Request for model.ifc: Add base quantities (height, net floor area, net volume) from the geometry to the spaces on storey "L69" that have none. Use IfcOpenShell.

First a look at what the model holds.

```python
import ifcopenshell
import ifcopenshell.util.element
import ifcopenshell.util.unit

model = ifcopenshell.open("model.ifc")
print(model.schema)
for unit_type in ("LENGTHUNIT", "AREAUNIT", "VOLUMEUNIT"):
    print(unit_type, ifcopenshell.util.unit.calculate_unit_scale(model, unit_type))
storey = next(s for s in model.by_type("IfcBuildingStorey") if s.Name == "L69")
spaces = [e for e in ifcopenshell.util.element.get_decomposition(storey) if e.is_a("IfcSpace")]
for e in sorted(spaces, key=lambda e: e.id()):
    print(e.id(), e.is_a(), e.Name, list(ifcopenshell.util.element.get_psets(e, qtos_only=True)), sep=" | ")
```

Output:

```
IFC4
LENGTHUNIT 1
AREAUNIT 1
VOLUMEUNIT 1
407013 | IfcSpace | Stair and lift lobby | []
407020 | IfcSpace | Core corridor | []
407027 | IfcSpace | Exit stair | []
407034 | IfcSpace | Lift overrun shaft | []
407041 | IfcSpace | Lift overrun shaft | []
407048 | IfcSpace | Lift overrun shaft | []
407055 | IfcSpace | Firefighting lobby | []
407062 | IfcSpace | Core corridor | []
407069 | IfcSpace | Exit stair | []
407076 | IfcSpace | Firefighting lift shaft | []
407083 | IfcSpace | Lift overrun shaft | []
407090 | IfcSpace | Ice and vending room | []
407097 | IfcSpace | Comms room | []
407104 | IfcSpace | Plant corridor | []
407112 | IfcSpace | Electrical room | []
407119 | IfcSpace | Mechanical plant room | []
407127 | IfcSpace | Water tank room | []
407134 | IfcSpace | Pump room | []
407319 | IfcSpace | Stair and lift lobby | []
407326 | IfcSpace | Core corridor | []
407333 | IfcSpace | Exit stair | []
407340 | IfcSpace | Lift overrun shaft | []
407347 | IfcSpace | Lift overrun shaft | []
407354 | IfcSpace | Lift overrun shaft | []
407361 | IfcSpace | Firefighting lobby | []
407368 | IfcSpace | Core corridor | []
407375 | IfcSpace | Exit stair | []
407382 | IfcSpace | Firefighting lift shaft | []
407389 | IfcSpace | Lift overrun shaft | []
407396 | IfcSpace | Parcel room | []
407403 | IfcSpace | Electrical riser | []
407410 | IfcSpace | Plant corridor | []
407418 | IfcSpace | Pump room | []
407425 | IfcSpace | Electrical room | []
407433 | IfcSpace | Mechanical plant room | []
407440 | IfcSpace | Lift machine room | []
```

```python
import ifcopenshell
import ifcopenshell.api.pset
import ifcopenshell.geom
import ifcopenshell.util.element
import ifcopenshell.util.shape
import ifcopenshell.util.unit

model = ifcopenshell.open("model.ifc")
unit_scale = ifcopenshell.util.unit.calculate_unit_scale(model)
area_scale = ifcopenshell.util.unit.calculate_unit_scale(model, "AREAUNIT")
volume_scale = ifcopenshell.util.unit.calculate_unit_scale(model, "VOLUMEUNIT")
settings = ifcopenshell.geom.settings()

storey = next(s for s in model.by_type("IfcBuildingStorey") if s.Name == "L69")
spaces = [e for e in ifcopenshell.util.element.get_decomposition(storey) if e.is_a("IfcSpace")]

for e in sorted(spaces, key=lambda e: e.id()):
    if ifcopenshell.util.element.get_psets(e, qtos_only=True, should_inherit=False):
        continue
    # Geometry comes back in metres, in the element's own axes.
    shape = ifcopenshell.geom.create_shape(settings, e)
    values = {
        "Height": ifcopenshell.util.shape.get_z(shape.geometry) / unit_scale,
        "NetFloorArea": ifcopenshell.util.shape.get_footprint_area(shape.geometry) / area_scale,
        "NetVolume": ifcopenshell.util.shape.get_volume(shape.geometry) / volume_scale,
    }
    qto = ifcopenshell.api.pset.add_qto(model, product=e, name="Qto_SpaceBaseQuantities")
    ifcopenshell.api.pset.edit_qto(model, qto=qto, properties=values)
    print(e.id(), {k: round(v, 3) for k, v in values.items()})

model.write("model_updated.ifc")
```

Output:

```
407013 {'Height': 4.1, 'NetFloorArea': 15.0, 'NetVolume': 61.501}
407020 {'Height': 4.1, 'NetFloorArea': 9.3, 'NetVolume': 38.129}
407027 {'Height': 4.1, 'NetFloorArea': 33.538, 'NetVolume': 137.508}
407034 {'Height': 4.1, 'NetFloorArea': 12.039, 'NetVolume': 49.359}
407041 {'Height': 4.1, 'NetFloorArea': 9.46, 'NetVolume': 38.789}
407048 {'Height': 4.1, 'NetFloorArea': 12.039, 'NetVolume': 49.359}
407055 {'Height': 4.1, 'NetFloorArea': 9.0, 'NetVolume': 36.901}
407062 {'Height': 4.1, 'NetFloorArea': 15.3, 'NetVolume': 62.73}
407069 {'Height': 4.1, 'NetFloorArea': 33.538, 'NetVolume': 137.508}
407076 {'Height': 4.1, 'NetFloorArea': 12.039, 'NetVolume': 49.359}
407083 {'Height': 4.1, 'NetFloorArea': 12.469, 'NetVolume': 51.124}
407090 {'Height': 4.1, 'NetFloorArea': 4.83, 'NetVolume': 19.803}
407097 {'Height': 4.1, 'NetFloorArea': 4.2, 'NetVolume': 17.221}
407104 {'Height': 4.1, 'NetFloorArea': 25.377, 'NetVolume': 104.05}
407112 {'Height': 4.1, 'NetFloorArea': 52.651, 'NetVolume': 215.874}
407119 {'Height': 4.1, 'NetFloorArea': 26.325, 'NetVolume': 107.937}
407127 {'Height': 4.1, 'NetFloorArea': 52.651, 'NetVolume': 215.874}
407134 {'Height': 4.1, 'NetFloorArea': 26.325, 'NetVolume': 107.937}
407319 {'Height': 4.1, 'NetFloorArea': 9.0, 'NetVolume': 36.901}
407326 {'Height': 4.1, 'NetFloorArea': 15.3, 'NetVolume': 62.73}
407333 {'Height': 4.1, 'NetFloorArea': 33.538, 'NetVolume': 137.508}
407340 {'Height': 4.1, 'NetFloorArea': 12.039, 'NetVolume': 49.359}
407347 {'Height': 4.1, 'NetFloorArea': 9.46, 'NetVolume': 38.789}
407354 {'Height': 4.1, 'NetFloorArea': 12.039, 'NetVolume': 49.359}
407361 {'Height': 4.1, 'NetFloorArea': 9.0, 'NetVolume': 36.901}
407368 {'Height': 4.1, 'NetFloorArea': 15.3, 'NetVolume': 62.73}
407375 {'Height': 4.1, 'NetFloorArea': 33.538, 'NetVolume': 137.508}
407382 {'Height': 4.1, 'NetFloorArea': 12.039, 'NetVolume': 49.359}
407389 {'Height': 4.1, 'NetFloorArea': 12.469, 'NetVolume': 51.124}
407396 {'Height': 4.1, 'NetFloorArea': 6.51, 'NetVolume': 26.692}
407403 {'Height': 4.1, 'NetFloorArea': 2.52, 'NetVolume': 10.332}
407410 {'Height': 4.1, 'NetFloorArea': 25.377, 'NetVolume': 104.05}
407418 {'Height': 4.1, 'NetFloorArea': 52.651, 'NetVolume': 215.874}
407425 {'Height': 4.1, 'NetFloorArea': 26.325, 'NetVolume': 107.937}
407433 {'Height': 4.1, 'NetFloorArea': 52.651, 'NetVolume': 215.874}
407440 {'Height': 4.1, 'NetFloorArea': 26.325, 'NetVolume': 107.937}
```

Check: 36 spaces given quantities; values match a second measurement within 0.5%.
